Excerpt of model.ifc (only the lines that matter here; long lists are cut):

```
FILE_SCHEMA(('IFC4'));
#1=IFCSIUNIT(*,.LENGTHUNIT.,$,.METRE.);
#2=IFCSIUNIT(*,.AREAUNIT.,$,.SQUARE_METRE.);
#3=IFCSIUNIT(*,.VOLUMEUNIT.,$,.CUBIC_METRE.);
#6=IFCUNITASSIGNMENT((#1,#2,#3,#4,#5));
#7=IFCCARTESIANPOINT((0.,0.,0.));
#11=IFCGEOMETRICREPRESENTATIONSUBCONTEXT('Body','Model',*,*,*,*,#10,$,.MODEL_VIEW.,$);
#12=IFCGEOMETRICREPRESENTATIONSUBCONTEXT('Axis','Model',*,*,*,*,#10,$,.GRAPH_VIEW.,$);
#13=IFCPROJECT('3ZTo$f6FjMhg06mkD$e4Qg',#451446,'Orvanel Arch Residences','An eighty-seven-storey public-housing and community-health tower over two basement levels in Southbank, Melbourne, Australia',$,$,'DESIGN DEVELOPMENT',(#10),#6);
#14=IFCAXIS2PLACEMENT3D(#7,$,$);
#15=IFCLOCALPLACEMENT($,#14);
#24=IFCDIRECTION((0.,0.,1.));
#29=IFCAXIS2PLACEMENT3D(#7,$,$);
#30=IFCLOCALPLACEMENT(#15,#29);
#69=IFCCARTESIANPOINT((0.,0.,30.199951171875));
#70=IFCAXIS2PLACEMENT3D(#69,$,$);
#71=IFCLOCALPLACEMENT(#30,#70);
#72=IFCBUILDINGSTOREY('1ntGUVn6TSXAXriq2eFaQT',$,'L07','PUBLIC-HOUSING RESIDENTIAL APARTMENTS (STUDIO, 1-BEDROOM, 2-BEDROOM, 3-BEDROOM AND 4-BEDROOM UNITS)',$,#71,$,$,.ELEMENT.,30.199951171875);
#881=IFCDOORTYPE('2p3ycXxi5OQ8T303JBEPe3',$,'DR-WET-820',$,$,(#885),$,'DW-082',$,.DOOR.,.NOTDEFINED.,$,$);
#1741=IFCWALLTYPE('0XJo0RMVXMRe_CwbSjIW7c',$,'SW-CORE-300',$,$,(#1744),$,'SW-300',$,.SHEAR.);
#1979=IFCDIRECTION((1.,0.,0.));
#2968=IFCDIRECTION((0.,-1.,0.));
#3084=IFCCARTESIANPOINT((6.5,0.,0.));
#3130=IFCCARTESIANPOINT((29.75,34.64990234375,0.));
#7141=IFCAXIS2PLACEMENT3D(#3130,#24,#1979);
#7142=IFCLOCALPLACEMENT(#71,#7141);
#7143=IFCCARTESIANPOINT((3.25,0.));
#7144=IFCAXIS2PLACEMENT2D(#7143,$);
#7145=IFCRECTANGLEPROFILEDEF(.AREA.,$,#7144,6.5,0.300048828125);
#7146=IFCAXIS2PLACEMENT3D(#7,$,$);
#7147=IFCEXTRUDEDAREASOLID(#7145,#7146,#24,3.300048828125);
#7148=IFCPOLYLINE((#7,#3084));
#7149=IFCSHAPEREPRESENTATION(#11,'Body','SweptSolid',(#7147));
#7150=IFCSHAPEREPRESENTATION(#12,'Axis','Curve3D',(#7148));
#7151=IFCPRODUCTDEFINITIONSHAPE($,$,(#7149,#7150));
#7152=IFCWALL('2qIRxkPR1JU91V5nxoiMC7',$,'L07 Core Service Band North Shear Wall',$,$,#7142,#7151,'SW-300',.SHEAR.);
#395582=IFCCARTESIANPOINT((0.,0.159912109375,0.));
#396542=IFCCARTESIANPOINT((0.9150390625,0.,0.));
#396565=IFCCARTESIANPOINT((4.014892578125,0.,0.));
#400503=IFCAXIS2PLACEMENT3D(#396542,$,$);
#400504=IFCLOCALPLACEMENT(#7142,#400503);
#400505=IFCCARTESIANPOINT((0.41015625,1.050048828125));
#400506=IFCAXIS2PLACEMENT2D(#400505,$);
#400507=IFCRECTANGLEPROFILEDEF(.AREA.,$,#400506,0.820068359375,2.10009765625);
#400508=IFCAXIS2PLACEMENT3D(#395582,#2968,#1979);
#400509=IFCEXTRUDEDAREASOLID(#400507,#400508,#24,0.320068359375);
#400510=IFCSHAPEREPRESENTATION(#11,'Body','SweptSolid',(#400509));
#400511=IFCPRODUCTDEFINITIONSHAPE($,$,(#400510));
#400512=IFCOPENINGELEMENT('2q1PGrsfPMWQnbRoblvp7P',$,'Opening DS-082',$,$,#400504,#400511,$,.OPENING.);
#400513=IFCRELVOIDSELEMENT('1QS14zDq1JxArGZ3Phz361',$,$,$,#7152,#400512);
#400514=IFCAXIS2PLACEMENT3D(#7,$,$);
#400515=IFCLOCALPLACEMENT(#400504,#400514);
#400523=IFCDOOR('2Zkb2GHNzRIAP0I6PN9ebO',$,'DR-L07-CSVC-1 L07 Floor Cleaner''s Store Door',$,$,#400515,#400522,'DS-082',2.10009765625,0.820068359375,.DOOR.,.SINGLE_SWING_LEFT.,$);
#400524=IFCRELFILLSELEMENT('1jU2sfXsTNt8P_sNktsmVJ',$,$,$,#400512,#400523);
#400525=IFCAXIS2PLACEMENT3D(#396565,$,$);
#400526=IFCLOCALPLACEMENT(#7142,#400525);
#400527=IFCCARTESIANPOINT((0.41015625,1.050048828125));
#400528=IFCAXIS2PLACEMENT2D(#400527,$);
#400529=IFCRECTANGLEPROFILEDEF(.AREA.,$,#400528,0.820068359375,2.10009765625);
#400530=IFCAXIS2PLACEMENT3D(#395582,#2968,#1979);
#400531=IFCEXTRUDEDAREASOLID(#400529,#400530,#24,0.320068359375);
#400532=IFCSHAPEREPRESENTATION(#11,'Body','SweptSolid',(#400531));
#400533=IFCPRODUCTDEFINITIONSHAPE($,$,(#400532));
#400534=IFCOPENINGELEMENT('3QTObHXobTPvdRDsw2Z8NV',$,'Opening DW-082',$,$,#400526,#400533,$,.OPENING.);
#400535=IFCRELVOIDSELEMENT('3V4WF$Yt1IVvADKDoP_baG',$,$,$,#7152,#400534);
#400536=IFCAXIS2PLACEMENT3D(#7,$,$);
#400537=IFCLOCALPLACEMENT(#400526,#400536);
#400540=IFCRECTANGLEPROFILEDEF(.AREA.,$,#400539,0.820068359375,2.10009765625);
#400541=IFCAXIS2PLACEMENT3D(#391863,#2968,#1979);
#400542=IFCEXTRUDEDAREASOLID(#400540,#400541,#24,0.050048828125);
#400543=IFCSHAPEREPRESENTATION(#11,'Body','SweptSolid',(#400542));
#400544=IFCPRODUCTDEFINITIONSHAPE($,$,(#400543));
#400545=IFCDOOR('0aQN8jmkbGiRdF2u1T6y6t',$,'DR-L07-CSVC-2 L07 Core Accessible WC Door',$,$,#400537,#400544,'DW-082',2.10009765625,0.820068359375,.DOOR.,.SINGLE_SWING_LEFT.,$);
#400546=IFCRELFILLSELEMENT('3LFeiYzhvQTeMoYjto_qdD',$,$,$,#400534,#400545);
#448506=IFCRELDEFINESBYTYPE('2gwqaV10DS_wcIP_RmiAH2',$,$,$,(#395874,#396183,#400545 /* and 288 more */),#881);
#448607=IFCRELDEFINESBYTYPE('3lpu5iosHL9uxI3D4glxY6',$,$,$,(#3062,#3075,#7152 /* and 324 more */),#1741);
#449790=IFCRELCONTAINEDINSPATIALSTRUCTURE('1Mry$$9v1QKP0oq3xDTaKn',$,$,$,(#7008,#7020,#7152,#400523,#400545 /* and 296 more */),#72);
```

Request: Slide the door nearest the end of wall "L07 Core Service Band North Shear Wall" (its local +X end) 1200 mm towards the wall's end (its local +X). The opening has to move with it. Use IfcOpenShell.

```python
import ifcopenshell
import ifcopenshell.api.geometry
import ifcopenshell.util.placement

model = ifcopenshell.open("model.ifc")

door = model.by_guid("0aQN8jmkbGiRdF2u1T6y6t")
opening = door.FillsVoids[0].RelatingOpeningElement
wall = opening.VoidsElements[0].RelatingBuildingElement

wall_matrix = ifcopenshell.util.placement.get_local_placement(wall.ObjectPlacement)
shift = wall_matrix[:3, 0] * 1.2
before = ifcopenshell.util.placement.get_local_placement(door.ObjectPlacement)[:3, 3].copy()

# The door is placed relative to its opening, so it follows when the opening moves.
matrix = ifcopenshell.util.placement.get_local_placement(opening.ObjectPlacement)
matrix[:3, 3] += shift
ifcopenshell.api.geometry.edit_object_placement(
    model, product=opening, matrix=matrix, is_si=False, should_transform_children=True
)

after = ifcopenshell.util.placement.get_local_placement(door.ObjectPlacement)[:3, 3]
print("door moved by", (after - before).round(3) + 0.0)

model.write("model_v2.ifc")
```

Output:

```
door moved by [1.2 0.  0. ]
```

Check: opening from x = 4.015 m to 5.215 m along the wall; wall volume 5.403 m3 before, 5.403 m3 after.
